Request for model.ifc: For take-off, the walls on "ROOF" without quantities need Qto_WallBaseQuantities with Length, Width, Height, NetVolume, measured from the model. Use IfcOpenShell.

First a look at what the model holds.

```python
import ifcopenshell
import ifcopenshell.util.element
import ifcopenshell.util.unit

model = ifcopenshell.open("model.ifc")
print(model.schema)
for unit_type in ("LENGTHUNIT", "AREAUNIT", "VOLUMEUNIT"):
    print(unit_type, ifcopenshell.util.unit.calculate_unit_scale(model, unit_type))
storey = next(s for s in model.by_type("IfcBuildingStorey") if s.Name == "ROOF")
walls = [e for e in ifcopenshell.util.element.get_decomposition(storey) if e.is_a("IfcWall")]
for e in sorted(walls, key=lambda e: e.id()):
    print(e.id(), e.is_a(), e.Name, list(ifcopenshell.util.element.get_psets(e, qtos_only=True)), sep=" | ")
```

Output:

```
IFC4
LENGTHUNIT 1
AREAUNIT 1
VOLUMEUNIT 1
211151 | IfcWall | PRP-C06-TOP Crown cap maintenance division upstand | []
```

```python
import ifcopenshell
import ifcopenshell.api.pset
import ifcopenshell.geom
import ifcopenshell.util.element
import ifcopenshell.util.shape
import ifcopenshell.util.unit

model = ifcopenshell.open("model.ifc")
unit_scale = ifcopenshell.util.unit.calculate_unit_scale(model)
volume_scale = ifcopenshell.util.unit.calculate_unit_scale(model, "VOLUMEUNIT")
settings = ifcopenshell.geom.settings()

storey = next(s for s in model.by_type("IfcBuildingStorey") if s.Name == "ROOF")
walls = [e for e in ifcopenshell.util.element.get_decomposition(storey) if e.is_a("IfcWall")]

for e in sorted(walls, key=lambda e: e.id()):
    if ifcopenshell.util.element.get_psets(e, qtos_only=True, should_inherit=False):
        continue
    # Geometry comes back in metres, in the element's own axes.
    shape = ifcopenshell.geom.create_shape(settings, e)
    values = {
        "Length": ifcopenshell.util.shape.get_x(shape.geometry) / unit_scale,
        "Width": ifcopenshell.util.shape.get_y(shape.geometry) / unit_scale,
        "Height": ifcopenshell.util.shape.get_z(shape.geometry) / unit_scale,
        "NetVolume": ifcopenshell.util.shape.get_volume(shape.geometry) / volume_scale,
    }
    qto = ifcopenshell.api.pset.add_qto(model, product=e, name="Qto_WallBaseQuantities")
    ifcopenshell.api.pset.edit_qto(model, qto=qto, properties=values)
    print(e.id(), {k: round(v, 3) for k, v in values.items()})

model.write("model_updated.ifc")
```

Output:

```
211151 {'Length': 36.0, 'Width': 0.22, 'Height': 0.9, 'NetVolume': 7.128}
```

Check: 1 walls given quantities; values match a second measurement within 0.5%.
